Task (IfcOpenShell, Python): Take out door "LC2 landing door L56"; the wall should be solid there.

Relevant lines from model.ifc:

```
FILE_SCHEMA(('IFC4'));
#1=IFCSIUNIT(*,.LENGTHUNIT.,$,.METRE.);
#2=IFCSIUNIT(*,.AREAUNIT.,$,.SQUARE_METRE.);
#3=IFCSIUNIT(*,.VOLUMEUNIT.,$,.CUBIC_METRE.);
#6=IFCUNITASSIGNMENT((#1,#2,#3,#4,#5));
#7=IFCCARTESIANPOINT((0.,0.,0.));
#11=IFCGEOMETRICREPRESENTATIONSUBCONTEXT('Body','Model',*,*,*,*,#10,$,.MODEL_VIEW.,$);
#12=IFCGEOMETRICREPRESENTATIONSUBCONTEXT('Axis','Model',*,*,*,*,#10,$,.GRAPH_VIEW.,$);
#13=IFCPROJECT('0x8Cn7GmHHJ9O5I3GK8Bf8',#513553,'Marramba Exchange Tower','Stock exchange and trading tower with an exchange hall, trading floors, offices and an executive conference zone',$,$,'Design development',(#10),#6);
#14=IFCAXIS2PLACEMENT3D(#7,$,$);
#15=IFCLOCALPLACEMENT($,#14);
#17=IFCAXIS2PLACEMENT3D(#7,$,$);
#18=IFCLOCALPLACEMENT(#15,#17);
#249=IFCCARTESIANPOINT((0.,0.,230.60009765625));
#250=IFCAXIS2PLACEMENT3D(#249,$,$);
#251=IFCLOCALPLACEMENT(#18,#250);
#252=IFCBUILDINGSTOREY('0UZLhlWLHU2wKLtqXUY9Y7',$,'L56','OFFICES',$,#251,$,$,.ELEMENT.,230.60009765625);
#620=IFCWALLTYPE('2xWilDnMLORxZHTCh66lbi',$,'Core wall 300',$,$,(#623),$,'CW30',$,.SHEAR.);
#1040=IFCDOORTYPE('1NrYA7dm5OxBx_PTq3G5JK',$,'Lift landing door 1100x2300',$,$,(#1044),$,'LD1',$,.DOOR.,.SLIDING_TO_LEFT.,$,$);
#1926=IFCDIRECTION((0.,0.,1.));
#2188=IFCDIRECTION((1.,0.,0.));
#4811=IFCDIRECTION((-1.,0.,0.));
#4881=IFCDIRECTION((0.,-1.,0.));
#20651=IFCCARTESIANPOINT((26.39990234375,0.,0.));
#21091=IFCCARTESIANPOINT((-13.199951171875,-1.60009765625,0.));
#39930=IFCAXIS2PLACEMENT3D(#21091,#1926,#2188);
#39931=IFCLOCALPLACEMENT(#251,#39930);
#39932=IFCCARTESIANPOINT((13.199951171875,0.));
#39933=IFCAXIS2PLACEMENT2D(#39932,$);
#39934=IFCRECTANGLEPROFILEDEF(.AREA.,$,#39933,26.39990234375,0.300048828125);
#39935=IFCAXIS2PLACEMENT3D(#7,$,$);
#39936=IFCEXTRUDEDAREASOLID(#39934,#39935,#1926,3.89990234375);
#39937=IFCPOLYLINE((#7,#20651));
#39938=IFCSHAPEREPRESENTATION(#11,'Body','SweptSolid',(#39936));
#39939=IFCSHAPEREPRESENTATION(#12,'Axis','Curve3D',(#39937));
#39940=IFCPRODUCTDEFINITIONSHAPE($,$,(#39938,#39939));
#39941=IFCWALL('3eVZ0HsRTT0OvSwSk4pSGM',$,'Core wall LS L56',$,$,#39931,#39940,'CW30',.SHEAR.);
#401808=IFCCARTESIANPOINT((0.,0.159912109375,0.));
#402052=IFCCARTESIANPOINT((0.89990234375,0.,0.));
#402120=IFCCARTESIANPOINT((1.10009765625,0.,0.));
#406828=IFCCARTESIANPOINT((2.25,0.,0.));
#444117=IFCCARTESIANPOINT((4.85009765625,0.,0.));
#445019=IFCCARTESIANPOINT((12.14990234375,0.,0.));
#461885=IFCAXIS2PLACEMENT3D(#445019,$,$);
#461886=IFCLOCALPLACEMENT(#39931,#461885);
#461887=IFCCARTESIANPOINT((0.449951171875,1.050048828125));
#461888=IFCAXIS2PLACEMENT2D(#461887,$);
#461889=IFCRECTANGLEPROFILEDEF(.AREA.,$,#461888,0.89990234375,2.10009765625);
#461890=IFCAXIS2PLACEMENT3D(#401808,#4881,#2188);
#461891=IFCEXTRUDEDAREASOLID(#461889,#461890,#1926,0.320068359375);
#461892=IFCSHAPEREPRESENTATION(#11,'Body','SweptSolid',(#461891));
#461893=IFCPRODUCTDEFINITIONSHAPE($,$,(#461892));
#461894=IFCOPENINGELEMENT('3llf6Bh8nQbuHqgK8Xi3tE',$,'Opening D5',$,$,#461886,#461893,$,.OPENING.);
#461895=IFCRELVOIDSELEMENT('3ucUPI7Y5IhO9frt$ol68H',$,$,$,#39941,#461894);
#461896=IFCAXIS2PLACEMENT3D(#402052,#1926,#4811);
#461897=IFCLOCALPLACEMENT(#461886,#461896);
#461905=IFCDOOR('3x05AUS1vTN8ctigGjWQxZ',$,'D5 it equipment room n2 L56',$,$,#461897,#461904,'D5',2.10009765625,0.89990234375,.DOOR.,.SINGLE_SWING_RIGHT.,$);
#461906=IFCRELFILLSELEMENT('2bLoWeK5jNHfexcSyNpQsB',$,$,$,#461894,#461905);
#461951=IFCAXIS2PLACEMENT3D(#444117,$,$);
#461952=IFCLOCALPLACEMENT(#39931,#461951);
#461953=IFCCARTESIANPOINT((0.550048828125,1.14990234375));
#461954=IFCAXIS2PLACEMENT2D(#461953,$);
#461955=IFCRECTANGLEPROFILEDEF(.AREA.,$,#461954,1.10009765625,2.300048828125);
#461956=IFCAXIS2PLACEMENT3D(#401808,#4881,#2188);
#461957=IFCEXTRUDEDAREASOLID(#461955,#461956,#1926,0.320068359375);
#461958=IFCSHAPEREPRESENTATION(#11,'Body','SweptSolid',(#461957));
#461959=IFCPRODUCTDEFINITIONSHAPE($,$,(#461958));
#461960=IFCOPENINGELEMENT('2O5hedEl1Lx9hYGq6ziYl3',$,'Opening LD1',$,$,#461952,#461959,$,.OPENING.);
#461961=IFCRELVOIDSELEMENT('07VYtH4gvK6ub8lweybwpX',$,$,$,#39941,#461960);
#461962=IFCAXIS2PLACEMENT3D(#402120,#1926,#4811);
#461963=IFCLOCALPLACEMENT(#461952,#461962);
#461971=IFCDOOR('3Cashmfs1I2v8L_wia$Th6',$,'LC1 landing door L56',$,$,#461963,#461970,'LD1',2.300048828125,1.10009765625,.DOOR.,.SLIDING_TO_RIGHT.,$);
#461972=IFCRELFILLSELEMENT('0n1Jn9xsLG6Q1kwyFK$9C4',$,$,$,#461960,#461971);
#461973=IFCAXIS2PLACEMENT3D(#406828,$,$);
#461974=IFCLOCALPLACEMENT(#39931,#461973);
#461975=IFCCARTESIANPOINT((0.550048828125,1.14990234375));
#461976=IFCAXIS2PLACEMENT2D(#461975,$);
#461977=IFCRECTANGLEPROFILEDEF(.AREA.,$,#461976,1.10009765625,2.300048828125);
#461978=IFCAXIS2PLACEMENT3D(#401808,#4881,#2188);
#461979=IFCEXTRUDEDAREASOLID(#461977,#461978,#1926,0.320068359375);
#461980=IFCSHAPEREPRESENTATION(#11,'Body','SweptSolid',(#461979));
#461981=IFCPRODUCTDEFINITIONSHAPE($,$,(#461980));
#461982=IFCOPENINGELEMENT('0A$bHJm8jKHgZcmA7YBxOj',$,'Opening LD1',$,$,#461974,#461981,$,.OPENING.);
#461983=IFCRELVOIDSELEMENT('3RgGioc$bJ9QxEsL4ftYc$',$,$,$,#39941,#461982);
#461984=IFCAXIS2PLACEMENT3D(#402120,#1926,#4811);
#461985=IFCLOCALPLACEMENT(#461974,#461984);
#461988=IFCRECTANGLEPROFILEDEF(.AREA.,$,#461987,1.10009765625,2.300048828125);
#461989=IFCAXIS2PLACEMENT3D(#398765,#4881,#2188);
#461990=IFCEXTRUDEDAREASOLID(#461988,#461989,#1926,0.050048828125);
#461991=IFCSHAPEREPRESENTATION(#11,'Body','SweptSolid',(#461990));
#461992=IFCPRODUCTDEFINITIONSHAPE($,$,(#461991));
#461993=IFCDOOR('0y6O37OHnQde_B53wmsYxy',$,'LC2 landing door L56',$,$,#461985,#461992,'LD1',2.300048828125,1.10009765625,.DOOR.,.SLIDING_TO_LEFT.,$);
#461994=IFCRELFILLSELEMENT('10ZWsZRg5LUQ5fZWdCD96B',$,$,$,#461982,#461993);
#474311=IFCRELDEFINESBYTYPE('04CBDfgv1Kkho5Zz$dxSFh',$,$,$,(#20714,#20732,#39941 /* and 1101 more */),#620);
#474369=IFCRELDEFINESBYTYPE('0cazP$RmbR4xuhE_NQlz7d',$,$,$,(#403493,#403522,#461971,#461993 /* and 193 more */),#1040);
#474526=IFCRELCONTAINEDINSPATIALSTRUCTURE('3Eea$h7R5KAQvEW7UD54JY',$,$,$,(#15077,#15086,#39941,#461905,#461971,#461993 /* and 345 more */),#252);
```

```python
import ifcopenshell
import ifcopenshell.api.feature
import ifcopenshell.api.root
import ifcopenshell.geom
import ifcopenshell.util.shape

model = ifcopenshell.open("model.ifc")
settings = ifcopenshell.geom.settings()


def volume(element):
    """Net volume in cubic metres, openings subtracted."""
    shape = ifcopenshell.geom.create_shape(settings, element)
    return ifcopenshell.util.shape.get_volume(shape.geometry)


door = model.by_id(461993)
opening = door.FillsVoids[0].RelatingOpeningElement
wall = opening.VoidsElements[0].RelatingBuildingElement
before = volume(wall)

ifcopenshell.api.root.remove_product(model, product=door)
ifcopenshell.api.feature.remove_feature(model, feature=opening)

after = volume(wall)

print(f"wall volume {before:.3f} -> {after:.3f} m3")

model.write("model_edited.ifc")
```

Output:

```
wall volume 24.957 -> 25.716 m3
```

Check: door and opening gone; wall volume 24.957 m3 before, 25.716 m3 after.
